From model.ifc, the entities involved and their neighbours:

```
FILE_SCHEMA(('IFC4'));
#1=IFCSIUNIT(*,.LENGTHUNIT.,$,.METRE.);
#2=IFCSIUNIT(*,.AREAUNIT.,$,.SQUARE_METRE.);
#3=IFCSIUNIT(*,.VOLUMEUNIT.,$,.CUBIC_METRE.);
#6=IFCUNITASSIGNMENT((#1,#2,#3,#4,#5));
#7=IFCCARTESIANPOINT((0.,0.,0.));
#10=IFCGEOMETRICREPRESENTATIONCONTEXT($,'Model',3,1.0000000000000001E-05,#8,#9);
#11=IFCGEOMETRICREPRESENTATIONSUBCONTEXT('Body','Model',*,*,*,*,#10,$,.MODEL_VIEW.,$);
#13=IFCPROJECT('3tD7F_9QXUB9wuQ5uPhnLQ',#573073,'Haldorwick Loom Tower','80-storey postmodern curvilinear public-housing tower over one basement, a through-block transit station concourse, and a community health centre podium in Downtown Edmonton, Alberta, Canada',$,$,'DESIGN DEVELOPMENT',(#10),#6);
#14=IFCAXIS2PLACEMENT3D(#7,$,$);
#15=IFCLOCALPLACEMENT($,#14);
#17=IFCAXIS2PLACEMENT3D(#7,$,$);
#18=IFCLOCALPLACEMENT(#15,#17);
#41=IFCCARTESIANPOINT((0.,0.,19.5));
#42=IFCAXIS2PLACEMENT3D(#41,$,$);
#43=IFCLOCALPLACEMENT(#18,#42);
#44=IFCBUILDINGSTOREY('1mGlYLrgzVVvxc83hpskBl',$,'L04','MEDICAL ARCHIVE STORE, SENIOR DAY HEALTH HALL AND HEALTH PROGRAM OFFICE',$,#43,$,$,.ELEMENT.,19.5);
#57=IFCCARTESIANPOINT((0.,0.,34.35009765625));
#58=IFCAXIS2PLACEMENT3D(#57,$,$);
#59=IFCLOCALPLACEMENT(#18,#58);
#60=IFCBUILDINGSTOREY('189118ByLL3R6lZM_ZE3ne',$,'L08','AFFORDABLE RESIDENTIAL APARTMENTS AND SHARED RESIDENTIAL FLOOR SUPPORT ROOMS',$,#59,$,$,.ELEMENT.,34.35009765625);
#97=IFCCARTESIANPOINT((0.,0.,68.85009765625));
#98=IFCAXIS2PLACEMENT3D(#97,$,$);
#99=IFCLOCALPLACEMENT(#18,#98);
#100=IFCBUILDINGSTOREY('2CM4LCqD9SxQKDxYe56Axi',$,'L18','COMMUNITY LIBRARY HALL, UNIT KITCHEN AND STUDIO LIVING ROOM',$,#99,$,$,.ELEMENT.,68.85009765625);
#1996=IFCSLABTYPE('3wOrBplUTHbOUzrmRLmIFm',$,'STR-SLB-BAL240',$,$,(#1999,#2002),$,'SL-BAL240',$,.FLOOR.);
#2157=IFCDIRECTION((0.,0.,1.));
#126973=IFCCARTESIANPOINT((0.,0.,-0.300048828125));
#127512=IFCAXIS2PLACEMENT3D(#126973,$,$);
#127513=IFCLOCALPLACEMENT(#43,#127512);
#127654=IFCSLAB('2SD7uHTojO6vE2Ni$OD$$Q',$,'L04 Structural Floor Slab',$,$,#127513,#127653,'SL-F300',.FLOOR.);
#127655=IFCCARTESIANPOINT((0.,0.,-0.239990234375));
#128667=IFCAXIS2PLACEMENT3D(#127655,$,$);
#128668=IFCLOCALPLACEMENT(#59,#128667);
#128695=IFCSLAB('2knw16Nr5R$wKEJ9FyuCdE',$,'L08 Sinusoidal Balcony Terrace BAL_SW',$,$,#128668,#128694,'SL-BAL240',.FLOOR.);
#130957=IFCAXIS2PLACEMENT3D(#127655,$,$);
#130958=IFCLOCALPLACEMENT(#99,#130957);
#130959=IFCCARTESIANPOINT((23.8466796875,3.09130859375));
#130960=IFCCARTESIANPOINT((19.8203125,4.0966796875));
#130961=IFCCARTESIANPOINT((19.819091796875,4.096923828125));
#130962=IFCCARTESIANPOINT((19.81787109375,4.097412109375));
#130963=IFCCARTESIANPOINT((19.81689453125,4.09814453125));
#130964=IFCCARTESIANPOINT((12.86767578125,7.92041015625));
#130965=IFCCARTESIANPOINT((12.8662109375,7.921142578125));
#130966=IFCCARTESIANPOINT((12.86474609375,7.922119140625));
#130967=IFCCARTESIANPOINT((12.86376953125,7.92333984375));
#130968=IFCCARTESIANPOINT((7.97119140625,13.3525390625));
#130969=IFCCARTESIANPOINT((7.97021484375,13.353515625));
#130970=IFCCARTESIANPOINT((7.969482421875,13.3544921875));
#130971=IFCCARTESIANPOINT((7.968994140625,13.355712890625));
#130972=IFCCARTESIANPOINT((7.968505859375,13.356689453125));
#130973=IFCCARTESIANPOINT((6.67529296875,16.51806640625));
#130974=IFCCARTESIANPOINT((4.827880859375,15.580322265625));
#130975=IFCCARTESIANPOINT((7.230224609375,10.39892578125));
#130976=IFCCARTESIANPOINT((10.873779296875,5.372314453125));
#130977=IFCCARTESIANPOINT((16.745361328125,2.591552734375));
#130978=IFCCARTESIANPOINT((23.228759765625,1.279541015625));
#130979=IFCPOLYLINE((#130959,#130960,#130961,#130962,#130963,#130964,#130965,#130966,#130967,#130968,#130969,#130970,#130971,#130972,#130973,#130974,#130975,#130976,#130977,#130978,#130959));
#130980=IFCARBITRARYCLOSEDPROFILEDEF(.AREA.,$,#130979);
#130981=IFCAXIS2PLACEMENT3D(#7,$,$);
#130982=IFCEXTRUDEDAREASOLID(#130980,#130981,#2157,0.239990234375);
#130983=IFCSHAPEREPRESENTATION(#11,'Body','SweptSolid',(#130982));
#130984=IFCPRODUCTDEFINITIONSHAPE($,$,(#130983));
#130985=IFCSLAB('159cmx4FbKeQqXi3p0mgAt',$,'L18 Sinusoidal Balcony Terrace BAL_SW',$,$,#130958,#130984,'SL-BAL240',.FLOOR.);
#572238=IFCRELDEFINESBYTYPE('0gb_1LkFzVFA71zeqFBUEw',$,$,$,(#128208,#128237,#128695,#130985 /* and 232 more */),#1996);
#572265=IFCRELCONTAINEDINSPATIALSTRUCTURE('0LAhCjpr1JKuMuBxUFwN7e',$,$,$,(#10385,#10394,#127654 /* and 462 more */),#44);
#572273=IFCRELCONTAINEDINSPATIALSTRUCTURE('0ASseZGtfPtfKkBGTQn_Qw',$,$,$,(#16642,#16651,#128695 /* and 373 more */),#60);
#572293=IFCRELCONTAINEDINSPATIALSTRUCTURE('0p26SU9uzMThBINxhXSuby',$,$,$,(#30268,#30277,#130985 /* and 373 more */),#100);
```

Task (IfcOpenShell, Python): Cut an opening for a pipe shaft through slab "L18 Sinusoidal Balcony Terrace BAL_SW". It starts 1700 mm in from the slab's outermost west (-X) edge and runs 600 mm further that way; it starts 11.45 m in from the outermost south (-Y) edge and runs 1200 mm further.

```python
import numpy as np
import ifcopenshell
import ifcopenshell.api.feature
import ifcopenshell.api.geometry
import ifcopenshell.api.root
import ifcopenshell.geom
import ifcopenshell.util.placement
import ifcopenshell.util.representation
import ifcopenshell.util.shape
import ifcopenshell.util.unit

model = ifcopenshell.open("model.ifc")
unit_scale = ifcopenshell.util.unit.calculate_unit_scale(model)
settings = ifcopenshell.geom.settings()


def volume(element):
    """Net volume in cubic metres, openings subtracted."""
    shape = ifcopenshell.geom.create_shape(settings, element)
    return ifcopenshell.util.shape.get_volume(shape.geometry)


slab = model.by_id(130985)
before = volume(slab)

# Extent in the slab's own axes, in metres. The edges named are its -X and -Y sides.
slab_shape = ifcopenshell.geom.create_shape(settings, slab)
vertices = ifcopenshell.util.shape.get_vertices(slab_shape.geometry)
x_min, y_min, bottom = vertices.min(axis=0)
top = vertices[:, 2].max()

opening = ifcopenshell.api.root.create_entity(model, ifc_class="IfcOpeningElement", name="Pipe shaft opening", predefined_type="OPENING")
context = ifcopenshell.util.representation.get_context(model, "Model", "Body", "MODEL_VIEW")
width, depth = 0.6, 1.2
outline = [(0.0, 0.0), (width, 0.0), (width, depth), (0.0, depth), (0.0, 0.0)]
# Overshoot both faces by 50 mm so the cut is clean.
shape = ifcopenshell.api.geometry.add_slab_representation(
    model, context=context, depth=top - bottom + 0.1, polyline=outline
)
ifcopenshell.api.geometry.assign_representation(model, product=opening, representation=shape)

matrix = ifcopenshell.util.placement.get_local_placement(slab.ObjectPlacement)
matrix[:, 3] = matrix @ np.append(np.array([x_min + 1.7, y_min + 11.45, bottom - 0.05]) / unit_scale, 1.0)
ifcopenshell.api.geometry.edit_object_placement(model, product=opening, matrix=matrix, is_si=False)
ifcopenshell.api.feature.add_feature(model, feature=opening, element=slab)

after = volume(slab)

print(f"slab volume {before:.3f} -> {after:.3f} m3")

model.write("model_rev.ifc")
```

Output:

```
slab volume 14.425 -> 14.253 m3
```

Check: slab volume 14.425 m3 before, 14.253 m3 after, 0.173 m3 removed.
